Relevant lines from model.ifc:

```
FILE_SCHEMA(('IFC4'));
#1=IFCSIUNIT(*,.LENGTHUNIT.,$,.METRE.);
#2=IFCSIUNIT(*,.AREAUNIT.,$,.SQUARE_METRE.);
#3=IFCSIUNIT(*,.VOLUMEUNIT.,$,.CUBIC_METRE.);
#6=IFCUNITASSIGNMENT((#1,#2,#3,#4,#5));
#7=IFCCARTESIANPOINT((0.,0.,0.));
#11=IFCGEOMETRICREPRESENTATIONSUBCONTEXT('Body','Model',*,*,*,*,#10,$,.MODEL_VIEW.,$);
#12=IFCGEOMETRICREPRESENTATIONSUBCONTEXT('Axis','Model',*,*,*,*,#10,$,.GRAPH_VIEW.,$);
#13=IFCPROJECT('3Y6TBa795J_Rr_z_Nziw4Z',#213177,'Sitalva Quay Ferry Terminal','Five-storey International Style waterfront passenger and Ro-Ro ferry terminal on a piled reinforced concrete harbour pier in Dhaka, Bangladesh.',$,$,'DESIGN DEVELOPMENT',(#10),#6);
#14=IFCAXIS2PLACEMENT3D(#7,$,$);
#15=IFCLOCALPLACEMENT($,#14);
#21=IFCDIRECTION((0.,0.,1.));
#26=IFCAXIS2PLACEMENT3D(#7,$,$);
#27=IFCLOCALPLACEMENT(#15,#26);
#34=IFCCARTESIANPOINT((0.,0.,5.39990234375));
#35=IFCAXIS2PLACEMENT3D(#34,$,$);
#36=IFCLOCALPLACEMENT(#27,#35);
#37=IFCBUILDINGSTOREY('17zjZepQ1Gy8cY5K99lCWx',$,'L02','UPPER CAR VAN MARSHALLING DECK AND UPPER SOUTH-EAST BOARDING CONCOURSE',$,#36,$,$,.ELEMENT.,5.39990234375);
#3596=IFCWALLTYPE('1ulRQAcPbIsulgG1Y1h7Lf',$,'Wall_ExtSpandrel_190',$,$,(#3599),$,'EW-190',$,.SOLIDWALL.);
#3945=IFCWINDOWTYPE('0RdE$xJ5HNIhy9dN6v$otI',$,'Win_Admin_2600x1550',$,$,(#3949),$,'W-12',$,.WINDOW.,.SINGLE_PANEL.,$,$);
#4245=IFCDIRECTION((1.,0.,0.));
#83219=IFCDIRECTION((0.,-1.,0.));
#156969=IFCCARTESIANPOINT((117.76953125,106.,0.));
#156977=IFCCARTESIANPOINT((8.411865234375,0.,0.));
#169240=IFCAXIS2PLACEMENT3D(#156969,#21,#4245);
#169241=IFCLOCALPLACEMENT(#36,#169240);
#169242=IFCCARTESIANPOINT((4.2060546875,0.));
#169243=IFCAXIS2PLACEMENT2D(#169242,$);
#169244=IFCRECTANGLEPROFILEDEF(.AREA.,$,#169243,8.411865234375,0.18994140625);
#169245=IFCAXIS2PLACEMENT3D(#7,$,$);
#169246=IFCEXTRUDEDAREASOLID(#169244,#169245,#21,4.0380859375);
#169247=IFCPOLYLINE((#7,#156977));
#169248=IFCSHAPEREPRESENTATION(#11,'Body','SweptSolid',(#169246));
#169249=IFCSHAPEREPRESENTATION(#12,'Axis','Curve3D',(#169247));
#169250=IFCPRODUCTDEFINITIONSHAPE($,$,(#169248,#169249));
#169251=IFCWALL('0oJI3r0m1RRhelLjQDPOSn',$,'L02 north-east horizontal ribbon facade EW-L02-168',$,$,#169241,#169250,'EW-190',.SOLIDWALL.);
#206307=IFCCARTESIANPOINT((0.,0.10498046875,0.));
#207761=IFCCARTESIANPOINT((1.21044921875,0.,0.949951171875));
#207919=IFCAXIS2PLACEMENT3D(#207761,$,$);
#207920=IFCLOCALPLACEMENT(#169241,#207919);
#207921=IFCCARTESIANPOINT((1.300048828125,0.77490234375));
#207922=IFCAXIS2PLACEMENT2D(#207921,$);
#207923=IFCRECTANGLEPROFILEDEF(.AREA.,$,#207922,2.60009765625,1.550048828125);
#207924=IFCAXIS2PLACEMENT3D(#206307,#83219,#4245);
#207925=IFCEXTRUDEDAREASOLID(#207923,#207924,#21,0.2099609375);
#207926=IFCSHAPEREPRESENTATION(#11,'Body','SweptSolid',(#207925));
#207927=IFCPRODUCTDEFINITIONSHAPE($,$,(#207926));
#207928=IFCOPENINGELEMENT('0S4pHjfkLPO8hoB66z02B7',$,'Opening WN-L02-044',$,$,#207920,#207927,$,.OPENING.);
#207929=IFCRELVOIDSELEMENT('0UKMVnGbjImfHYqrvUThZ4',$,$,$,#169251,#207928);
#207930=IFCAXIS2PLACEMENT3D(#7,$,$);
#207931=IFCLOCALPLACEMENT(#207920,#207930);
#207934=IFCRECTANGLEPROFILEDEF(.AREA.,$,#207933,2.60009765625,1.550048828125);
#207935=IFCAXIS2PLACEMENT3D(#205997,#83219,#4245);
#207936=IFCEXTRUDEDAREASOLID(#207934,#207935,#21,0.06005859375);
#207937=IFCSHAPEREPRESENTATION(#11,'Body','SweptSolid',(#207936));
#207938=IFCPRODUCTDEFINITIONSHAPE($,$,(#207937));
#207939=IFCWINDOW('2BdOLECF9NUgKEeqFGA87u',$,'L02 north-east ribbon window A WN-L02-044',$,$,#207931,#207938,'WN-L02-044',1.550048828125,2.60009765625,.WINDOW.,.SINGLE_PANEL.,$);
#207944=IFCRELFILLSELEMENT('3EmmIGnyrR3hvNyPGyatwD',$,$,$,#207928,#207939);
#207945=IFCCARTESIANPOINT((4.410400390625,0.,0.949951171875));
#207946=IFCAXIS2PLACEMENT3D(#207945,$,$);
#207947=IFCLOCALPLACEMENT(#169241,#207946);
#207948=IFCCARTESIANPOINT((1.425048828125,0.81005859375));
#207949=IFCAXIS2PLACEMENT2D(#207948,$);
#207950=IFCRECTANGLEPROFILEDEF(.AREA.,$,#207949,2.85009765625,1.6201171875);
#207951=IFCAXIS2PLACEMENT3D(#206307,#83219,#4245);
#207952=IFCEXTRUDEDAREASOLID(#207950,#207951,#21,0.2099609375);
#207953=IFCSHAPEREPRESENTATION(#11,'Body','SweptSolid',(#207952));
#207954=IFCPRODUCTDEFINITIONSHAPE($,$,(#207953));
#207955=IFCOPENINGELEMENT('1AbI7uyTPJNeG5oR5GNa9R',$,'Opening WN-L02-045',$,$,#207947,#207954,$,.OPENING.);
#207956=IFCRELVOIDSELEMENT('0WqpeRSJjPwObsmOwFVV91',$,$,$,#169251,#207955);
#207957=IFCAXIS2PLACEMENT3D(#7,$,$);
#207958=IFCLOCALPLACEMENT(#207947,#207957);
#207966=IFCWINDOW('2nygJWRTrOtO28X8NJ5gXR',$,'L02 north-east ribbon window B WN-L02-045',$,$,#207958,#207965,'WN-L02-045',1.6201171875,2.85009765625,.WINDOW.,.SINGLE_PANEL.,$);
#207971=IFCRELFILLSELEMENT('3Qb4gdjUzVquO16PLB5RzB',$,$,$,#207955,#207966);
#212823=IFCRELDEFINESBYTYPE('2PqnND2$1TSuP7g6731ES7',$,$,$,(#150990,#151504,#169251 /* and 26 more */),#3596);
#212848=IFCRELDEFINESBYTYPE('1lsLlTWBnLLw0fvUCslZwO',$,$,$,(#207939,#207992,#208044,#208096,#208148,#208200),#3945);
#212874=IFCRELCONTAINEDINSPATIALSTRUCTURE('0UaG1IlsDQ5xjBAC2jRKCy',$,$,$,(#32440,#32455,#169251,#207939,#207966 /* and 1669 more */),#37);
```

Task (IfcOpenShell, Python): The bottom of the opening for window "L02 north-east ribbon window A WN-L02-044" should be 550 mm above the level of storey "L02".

```python
import numpy as np
import ifcopenshell
import ifcopenshell.api.geometry
import ifcopenshell.geom
import ifcopenshell.util.element
import ifcopenshell.util.placement
import ifcopenshell.util.shape
import ifcopenshell.util.unit

model = ifcopenshell.open("model.ifc")
unit_scale = ifcopenshell.util.unit.calculate_unit_scale(model)

window = model.by_guid("2BdOLECF9NUgKEeqFGA87u")
opening = window.FillsVoids[0].RelatingOpeningElement
storey = ifcopenshell.util.element.get_container(window, ifc_class="IfcBuildingStorey")
level = ifcopenshell.util.placement.get_local_placement(storey.ObjectPlacement)[2, 3]

# The opening's origin need not be at the sill, so measure its lowest point.
shape = ifcopenshell.geom.create_shape(ifcopenshell.geom.settings(), opening)
bottom = ifcopenshell.util.shape.get_shape_bottom_elevation(shape, shape.geometry) / unit_scale
dz = level + 0.55 / unit_scale - bottom

shift = np.array([0.0, 0.0, dz])
# The window is placed relative to its opening, so it follows when the opening moves.
matrix = ifcopenshell.util.placement.get_local_placement(opening.ObjectPlacement)
matrix[:3, 3] += shift
ifcopenshell.api.geometry.edit_object_placement(
    model, product=opening, matrix=matrix, is_si=False, should_transform_children=True
)

print(f"moved by {dz * unit_scale:+.3f} m")

model.write("model_rev.ifc")
```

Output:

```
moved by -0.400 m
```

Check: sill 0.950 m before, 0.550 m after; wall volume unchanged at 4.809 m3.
